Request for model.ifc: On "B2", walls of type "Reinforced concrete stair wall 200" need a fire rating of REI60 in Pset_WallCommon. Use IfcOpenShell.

First a look at what the model holds.

```python
import ifcopenshell
import ifcopenshell.util.element

model = ifcopenshell.open("model.ifc")
print(model.schema)
storey = next(s for s in model.by_type("IfcBuildingStorey") if s.Name == "B2")
walls = [e for e in ifcopenshell.util.element.get_decomposition(storey) if e.is_a("IfcWall")]
seen = {}
for e in walls:
    element_type = ifcopenshell.util.element.get_type(e)
    key = (element_type.Name if element_type != e and element_type else None, ifcopenshell.util.element.get_pset(e, "Pset_WallCommon", "FireRating"))
    seen[key] = seen.get(key, 0) + 1
for (name, value), count in sorted(seen.items(), key=str):
    print(count, "x", name, "|", value)
```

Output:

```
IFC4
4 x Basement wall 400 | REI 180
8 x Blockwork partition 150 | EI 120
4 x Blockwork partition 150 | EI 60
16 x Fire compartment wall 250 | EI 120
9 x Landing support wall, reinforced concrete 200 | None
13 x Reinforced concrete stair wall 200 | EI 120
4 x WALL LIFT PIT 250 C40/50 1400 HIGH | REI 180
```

```python
import ifcopenshell
import ifcopenshell.api.pset
import ifcopenshell.util.element

model = ifcopenshell.open("model.ifc")

storey = next(s for s in model.by_type("IfcBuildingStorey") if s.Name == "B2")
walls = [e for e in ifcopenshell.util.element.get_decomposition(storey) if e.is_a("IfcWall")]

count = 0
for e in walls:
    element_type = ifcopenshell.util.element.get_type(e)
    if element_type in (None, e) or element_type.Name != "Reinforced concrete stair wall 200":
        continue
    found = ifcopenshell.util.element.get_pset(e, "Pset_WallCommon", should_inherit=False)
    if found:
        pset = model.by_id(found["id"])
        if len(ifcopenshell.util.element.get_elements_by_pset(pset)) > 1:
            pset = ifcopenshell.api.pset.unshare_pset(model, products=[e], pset=pset)[0]
    else:
        pset = ifcopenshell.api.pset.add_pset(model, product=e, name="Pset_WallCommon")
    ifcopenshell.api.pset.edit_pset(model, pset=pset, properties={"FireRating": "REI60"})
    count += 1

print(count, "walls updated")

model.write("model_rev.ifc")
```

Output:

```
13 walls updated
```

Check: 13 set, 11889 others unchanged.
